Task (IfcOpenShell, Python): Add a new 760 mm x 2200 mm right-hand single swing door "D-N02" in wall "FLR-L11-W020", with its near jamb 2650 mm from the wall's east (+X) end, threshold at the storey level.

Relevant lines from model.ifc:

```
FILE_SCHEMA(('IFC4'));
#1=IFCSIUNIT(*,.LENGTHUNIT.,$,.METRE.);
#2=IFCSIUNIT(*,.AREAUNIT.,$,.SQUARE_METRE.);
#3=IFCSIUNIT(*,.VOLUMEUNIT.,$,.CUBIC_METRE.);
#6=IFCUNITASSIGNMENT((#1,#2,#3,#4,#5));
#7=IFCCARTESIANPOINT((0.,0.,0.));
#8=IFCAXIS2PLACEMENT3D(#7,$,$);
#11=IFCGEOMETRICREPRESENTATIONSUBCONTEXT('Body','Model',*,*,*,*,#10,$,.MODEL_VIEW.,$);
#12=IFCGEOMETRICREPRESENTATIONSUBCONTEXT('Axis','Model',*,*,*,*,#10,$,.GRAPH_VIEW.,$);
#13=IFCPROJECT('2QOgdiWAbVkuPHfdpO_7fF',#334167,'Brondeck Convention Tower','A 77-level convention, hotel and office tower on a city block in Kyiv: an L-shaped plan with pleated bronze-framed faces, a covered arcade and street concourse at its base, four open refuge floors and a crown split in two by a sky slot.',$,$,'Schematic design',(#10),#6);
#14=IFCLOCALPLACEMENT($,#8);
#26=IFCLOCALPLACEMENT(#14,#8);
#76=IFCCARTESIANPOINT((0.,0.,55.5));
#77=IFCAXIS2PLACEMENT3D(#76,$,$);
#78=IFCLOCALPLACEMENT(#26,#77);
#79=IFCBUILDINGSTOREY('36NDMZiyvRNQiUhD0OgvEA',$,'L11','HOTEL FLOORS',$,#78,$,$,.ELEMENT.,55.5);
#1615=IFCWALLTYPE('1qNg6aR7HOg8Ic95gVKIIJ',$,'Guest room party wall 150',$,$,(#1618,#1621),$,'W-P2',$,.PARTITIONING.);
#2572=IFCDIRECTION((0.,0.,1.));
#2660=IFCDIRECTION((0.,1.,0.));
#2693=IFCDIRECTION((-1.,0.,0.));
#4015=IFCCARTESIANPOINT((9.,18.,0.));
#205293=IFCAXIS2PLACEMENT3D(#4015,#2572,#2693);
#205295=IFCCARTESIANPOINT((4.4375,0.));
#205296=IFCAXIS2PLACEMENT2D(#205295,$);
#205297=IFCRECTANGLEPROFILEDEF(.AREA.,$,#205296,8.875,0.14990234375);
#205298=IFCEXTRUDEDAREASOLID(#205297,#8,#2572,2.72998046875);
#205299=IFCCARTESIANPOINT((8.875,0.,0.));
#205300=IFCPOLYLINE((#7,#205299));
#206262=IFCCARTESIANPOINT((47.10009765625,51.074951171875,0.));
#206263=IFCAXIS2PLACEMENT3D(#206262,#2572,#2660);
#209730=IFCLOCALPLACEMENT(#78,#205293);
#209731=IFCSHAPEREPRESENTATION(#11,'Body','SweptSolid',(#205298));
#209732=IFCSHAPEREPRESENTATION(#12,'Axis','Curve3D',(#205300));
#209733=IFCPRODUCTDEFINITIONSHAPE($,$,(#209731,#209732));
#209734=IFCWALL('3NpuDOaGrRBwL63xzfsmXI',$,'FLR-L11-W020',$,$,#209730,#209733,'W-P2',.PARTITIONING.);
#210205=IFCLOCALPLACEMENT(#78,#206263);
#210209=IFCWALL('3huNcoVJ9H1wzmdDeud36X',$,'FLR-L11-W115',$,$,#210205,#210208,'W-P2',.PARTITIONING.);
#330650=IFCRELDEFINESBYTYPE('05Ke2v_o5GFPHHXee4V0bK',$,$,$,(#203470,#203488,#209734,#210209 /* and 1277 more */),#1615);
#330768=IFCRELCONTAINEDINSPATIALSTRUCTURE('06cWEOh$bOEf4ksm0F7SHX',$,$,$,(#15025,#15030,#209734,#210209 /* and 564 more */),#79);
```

```python
import numpy as np
import ifcopenshell
import ifcopenshell.api.feature
import ifcopenshell.api.geometry
import ifcopenshell.api.root
import ifcopenshell.api.spatial
import ifcopenshell.geom
import ifcopenshell.util.element
import ifcopenshell.util.placement
import ifcopenshell.util.representation
import ifcopenshell.util.shape
import ifcopenshell.util.unit

model = ifcopenshell.open("model.ifc")
unit_scale = ifcopenshell.util.unit.calculate_unit_scale(model)
settings = ifcopenshell.geom.settings()


def volume(element):
    """Net volume in cubic metres, openings subtracted."""
    shape = ifcopenshell.geom.create_shape(settings, element)
    return ifcopenshell.util.shape.get_volume(shape.geometry)


wall = model.by_guid("3NpuDOaGrRBwL63xzfsmXI")
storey = ifcopenshell.util.element.get_container(wall, ifc_class="IfcBuildingStorey")
context = ifcopenshell.util.representation.get_context(model, "Model", "Body", "MODEL_VIEW")
before = volume(wall)

width, height, from_end, sill = 0.76, 2.2, 2.65, 0.0  # metres

# The wall runs along its own X axis, and the end named is its -X end.
wall_shape = ifcopenshell.geom.create_shape(settings, wall)
x, y, z = ifcopenshell.util.shape.get_vertices(wall_shape.geometry).T
start = x.min() + from_end
face, thickness = float(y.min()), float(y.max() - y.min())
wall_matrix = ifcopenshell.util.placement.get_local_placement(wall.ObjectPlacement)
level = ifcopenshell.util.placement.get_local_placement(storey.ObjectPlacement)[2, 3]


def in_wall(x, y):
    """Placement at x, y metres in the wall's axes, at sill height."""
    matrix = wall_matrix.copy()
    matrix[:, 3] = wall_matrix @ np.array([x / unit_scale, y / unit_scale, 0.0, 1.0])
    matrix[2, 3] = level + sill / unit_scale
    return matrix


# Opening: a box that overshoots both wall faces by 50 mm.
opening = ifcopenshell.api.root.create_entity(model, ifc_class="IfcOpeningElement", predefined_type="OPENING")
box = ifcopenshell.api.geometry.add_wall_representation(
    model, context=context, length=width, height=height, thickness=thickness + 0.1
)
ifcopenshell.api.geometry.assign_representation(model, product=opening, representation=box)
ifcopenshell.api.geometry.edit_object_placement(model, product=opening, matrix=in_wall(start, face - 0.05), is_si=False)
ifcopenshell.api.feature.add_feature(model, feature=opening, element=wall)

door = ifcopenshell.api.root.create_entity(model, ifc_class="IfcDoor", name="D-N02", predefined_type="DOOR")
door.OverallWidth, door.OverallHeight = width / unit_scale, height / unit_scale
door.OperationType = "SINGLE_SWING_RIGHT"
body = ifcopenshell.api.geometry.add_door_representation(
    model,
    context=context,
    overall_width=door.OverallWidth,
    overall_height=door.OverallHeight,
    operation_type="SINGLE_SWING_RIGHT",
    lining_properties={"LiningDepth": thickness / unit_scale, "ThresholdDepth": thickness / unit_scale},
)
ifcopenshell.api.geometry.assign_representation(model, product=door, representation=body)
ifcopenshell.api.spatial.assign_container(model, products=[door], relating_structure=storey)
ifcopenshell.api.feature.add_filling(model, opening=opening, element=door)

# The lining spans the wall, so the door starts at the wall face.
ifcopenshell.api.geometry.edit_object_placement(model, product=door, matrix=in_wall(start, face), is_si=False)

after = volume(wall)

print(f"wall volume {before:.3f} -> {after:.3f} m3")

model.write("model_edited.ifc")
```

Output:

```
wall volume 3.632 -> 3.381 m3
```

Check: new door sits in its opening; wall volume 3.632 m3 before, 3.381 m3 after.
